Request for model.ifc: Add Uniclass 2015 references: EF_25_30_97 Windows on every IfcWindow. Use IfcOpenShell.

First a look at what the model holds.

```python
import ifcopenshell

model = ifcopenshell.open("model.ifc")
print(model.schema)
print("classifications:", [c.Name for c in model.by_type("IfcClassification")])
for ifc_class in ("IfcDoor", "IfcRoof", "IfcStair", "IfcWall", "IfcWindow"):
    print(ifc_class, len(model.by_type(ifc_class)))
```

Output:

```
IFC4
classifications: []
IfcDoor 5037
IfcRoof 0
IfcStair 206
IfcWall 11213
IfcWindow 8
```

```python
import ifcopenshell
import ifcopenshell.api.classification

model = ifcopenshell.open("model.ifc")

system = ifcopenshell.api.classification.add_classification(model, classification="Uniclass 2015")

codes = {
    "IfcWindow": ("EF_25_30_97", "Windows"),
}
for ifc_class, (code, name) in codes.items():
    products = model.by_type(ifc_class)
    ifcopenshell.api.classification.add_reference(
        model, products=products, classification=system, identification=code, name=name
    )
    print(code, len(products))

model.write("model_edited.ifc")
```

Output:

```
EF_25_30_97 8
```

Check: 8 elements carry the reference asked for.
